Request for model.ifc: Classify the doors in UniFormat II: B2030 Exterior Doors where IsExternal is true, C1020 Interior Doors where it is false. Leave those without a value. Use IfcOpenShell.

First a look at what the model holds.

```python
import ifcopenshell
import ifcopenshell.util.element

model = ifcopenshell.open("model.ifc")
print(model.schema)
print("classifications:", [c.Name for c in model.by_type("IfcClassification")])
values = [ifcopenshell.util.element.get_pset(e, "Pset_DoorCommon", "IsExternal") for e in model.by_type("IfcDoor")]
for value in (True, False, None):
    print("IsExternal", value, values.count(value))
```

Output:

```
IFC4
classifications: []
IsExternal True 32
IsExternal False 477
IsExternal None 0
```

```python
import ifcopenshell
import ifcopenshell.api.classification
import ifcopenshell.util.element

model = ifcopenshell.open("model.ifc")

system = ifcopenshell.api.classification.add_classification(model, classification="UniFormat II")

doors = model.by_type("IfcDoor")
external = {e: ifcopenshell.util.element.get_pset(e, "Pset_DoorCommon", "IsExternal") for e in doors}
for flag, code, name in ((True, "B2030", "Exterior Doors"), (False, "C1020", "Interior Doors")):
    products = [e for e in doors if external[e] is flag]
    ifcopenshell.api.classification.add_reference(
        model, products=products, classification=system, identification=code, name=name
    )
    print(code, len(products))

model.write("model_rev.ifc")
```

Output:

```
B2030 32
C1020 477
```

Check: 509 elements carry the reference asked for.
